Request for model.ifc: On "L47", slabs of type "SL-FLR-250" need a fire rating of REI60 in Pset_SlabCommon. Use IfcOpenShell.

First a look at what the model holds.

```python
import ifcopenshell
import ifcopenshell.util.element

model = ifcopenshell.open("model.ifc")
print(model.schema)
storey = next(s for s in model.by_type("IfcBuildingStorey") if s.Name == "L47")
slabs = [e for e in ifcopenshell.util.element.get_decomposition(storey) if e.is_a("IfcSlab")]
seen = {}
for e in slabs:
    element_type = ifcopenshell.util.element.get_type(e)
    key = (element_type.Name if element_type != e and element_type else None, ifcopenshell.util.element.get_pset(e, "Pset_SlabCommon", "FireRating"))
    seen[key] = seen.get(key, 0) + 1
for (name, value), count in sorted(seen.items(), key=str):
    print(count, "x", name, "|", value)
```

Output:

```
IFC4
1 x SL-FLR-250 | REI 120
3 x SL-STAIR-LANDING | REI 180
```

```python
import ifcopenshell
import ifcopenshell.api.pset
import ifcopenshell.util.element

model = ifcopenshell.open("model.ifc")

storey = next(s for s in model.by_type("IfcBuildingStorey") if s.Name == "L47")
slabs = [e for e in ifcopenshell.util.element.get_decomposition(storey) if e.is_a("IfcSlab")]

count = 0
for e in slabs:
    element_type = ifcopenshell.util.element.get_type(e)
    if element_type in (None, e) or element_type.Name != "SL-FLR-250":
        continue
    # add_pset returns the element's existing set when there is one.
    pset = ifcopenshell.api.pset.add_pset(model, product=e, name="Pset_SlabCommon")
    ifcopenshell.api.pset.edit_pset(model, pset=pset, properties={"FireRating": "REI60"})
    count += 1

print(count, "slabs updated")

model.write("model-out.ifc")
```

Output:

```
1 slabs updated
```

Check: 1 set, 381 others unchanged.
